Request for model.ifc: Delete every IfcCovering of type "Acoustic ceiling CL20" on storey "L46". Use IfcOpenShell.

First a look at what the model holds.

```python
import ifcopenshell
import ifcopenshell.util.element

model = ifcopenshell.open("model.ifc")
print(model.schema)
storey = next(s for s in model.by_type("IfcBuildingStorey") if s.Name == "L46")
coverings = [e for e in ifcopenshell.util.element.get_decomposition(storey) if e.is_a("IfcCovering")]
seen = {}
for e in coverings:
    element_type = ifcopenshell.util.element.get_type(e)
    name = element_type.Name if element_type not in (None, e) else None
    seen[name] = seen.get(name, 0) + 1
for name, count in sorted(seen.items(), key=str):
    print(count, "x", name)
```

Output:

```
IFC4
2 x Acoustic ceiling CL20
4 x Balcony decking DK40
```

```python
import ifcopenshell
import ifcopenshell.api.root
import ifcopenshell.util.element

model = ifcopenshell.open("model.ifc")

storey = next(s for s in model.by_type("IfcBuildingStorey") if s.Name == "L46")
coverings = [e for e in ifcopenshell.util.element.get_decomposition(storey) if e.is_a("IfcCovering")]
targets = [e for e in coverings if (t := ifcopenshell.util.element.get_type(e)) not in (None, e) and t.Name == "Acoustic ceiling CL20"]

for e in targets:
    ifcopenshell.api.root.remove_product(model, product=e)
print(len(targets), "removed")

model.write("model_updated.ifc")
```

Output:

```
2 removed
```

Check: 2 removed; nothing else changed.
